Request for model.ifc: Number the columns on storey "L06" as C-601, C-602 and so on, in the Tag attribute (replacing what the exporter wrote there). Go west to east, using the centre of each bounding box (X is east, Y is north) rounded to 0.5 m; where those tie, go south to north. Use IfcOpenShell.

First a look at what the model holds.

```python
import ifcopenshell
import ifcopenshell.util.element
import ifcopenshell.util.placement

model = ifcopenshell.open("model.ifc")
print(model.schema)
storey = next(s for s in model.by_type("IfcBuildingStorey") if s.Name == "L06")
columns = [e for e in ifcopenshell.util.element.get_decomposition(storey) if e.is_a("IfcColumn")]
for e in sorted(columns, key=lambda e: e.id()):
    origin = ifcopenshell.util.placement.get_local_placement(e.ObjectPlacement)[:3, 3]
    print(e.id(), e.Tag, e.Name, origin.round(2) + 0.0, sep=" | ")
```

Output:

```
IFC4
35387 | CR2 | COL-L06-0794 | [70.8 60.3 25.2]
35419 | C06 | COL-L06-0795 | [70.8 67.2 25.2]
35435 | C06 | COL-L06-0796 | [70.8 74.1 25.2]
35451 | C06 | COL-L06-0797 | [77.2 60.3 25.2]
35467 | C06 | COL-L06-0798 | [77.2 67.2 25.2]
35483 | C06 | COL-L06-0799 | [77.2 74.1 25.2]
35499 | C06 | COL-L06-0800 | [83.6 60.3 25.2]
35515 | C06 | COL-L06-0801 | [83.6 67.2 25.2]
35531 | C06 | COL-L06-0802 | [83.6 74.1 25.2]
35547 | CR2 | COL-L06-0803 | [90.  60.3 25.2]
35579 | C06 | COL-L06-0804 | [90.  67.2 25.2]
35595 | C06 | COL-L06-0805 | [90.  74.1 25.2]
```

```python
import ifcopenshell
import ifcopenshell.geom
import ifcopenshell.util.element
import ifcopenshell.util.shape

model = ifcopenshell.open("model.ifc")
settings = ifcopenshell.geom.settings()
settings.set("use-world-coords", True)


def centre(element):
    shape = ifcopenshell.geom.create_shape(settings, element)
    return ifcopenshell.util.shape.get_bbox_centroid(shape.geometry)


storey = next(s for s in model.by_type("IfcBuildingStorey") if s.Name == "L06")
columns = [e for e in ifcopenshell.util.element.get_decomposition(storey) if e.is_a("IfcColumn")]

# Insertion points can sit at a corner or the storey origin, so sort by the geometry (in metres).
centres = {e: centre(e) for e in columns}
columns.sort(key=lambda e: (round(centres[e][0] / 0.5), centres[e][1]))

for i, e in enumerate(columns, start=1):
    number = f"C-6{i:02d}"
    e.Tag = number
    print(e.id(), number)

model.write("model-out.ifc")
```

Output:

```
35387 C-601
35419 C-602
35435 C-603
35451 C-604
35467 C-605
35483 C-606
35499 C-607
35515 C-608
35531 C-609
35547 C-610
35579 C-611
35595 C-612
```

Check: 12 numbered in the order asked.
